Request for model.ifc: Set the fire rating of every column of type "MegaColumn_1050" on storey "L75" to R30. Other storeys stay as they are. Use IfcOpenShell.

First a look at what the model holds.

```python
import ifcopenshell
import ifcopenshell.util.element

model = ifcopenshell.open("model.ifc")
print(model.schema)
storey = next(s for s in model.by_type("IfcBuildingStorey") if s.Name == "L75")
columns = [e for e in ifcopenshell.util.element.get_decomposition(storey) if e.is_a("IfcColumn")]
seen = {}
for e in columns:
    element_type = ifcopenshell.util.element.get_type(e)
    key = (element_type.Name if element_type != e and element_type else None, ifcopenshell.util.element.get_pset(e, "Pset_ColumnCommon", "FireRating"))
    seen[key] = seen.get(key, 0) + 1
for (name, value), count in sorted(seen.items(), key=str):
    print(count, "x", name, "|", value)
```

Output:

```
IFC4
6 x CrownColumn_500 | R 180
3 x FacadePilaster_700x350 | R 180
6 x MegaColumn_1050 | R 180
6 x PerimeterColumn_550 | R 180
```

```python
import ifcopenshell
import ifcopenshell.api.pset
import ifcopenshell.util.element

model = ifcopenshell.open("model.ifc")

storey = next(s for s in model.by_type("IfcBuildingStorey") if s.Name == "L75")
columns = [e for e in ifcopenshell.util.element.get_decomposition(storey) if e.is_a("IfcColumn")]

count = 0
for e in columns:
    element_type = ifcopenshell.util.element.get_type(e)
    if element_type in (None, e) or element_type.Name != "MegaColumn_1050":
        continue
    # add_pset returns the element's existing set when there is one.
    pset = ifcopenshell.api.pset.add_pset(model, product=e, name="Pset_ColumnCommon")
    ifcopenshell.api.pset.edit_pset(model, pset=pset, properties={"FireRating": "R30"})
    count += 1

print(count, "columns updated")

model.write("model-out.ifc")
```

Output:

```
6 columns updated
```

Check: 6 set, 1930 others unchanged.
